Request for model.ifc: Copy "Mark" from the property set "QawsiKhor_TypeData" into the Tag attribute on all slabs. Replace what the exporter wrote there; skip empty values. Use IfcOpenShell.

First a look at what the model holds.

```python
import ifcopenshell
import ifcopenshell.util.element

model = ifcopenshell.open("model.ifc")
print(model.schema)
slabs = model.by_type("IfcSlab")
print(len(slabs), "slabs")
for e in slabs[:8]:
    source = ifcopenshell.util.element.get_pset(e, "QawsiKhor_TypeData", "Mark")
    target = e.Tag
    print(e.id(), repr(source), repr(target), sep=" | ")
```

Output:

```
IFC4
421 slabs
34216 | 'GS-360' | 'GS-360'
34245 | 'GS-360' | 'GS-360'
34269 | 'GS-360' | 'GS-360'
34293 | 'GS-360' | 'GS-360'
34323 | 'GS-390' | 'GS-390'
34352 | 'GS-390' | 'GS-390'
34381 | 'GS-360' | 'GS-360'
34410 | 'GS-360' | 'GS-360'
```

```python
import ifcopenshell
import ifcopenshell.util.element

model = ifcopenshell.open("model.ifc")

count = 0
for e in model.by_type("IfcSlab"):
    value = ifcopenshell.util.element.get_pset(e, "QawsiKhor_TypeData", "Mark")
    current = e.Tag
    if not value or not value.strip() or current == value:
        continue
    e.Tag = value
    count += 1

print(count, "slabs updated")

model.write("model_v2.ifc")
```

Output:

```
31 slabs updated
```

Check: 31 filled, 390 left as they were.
